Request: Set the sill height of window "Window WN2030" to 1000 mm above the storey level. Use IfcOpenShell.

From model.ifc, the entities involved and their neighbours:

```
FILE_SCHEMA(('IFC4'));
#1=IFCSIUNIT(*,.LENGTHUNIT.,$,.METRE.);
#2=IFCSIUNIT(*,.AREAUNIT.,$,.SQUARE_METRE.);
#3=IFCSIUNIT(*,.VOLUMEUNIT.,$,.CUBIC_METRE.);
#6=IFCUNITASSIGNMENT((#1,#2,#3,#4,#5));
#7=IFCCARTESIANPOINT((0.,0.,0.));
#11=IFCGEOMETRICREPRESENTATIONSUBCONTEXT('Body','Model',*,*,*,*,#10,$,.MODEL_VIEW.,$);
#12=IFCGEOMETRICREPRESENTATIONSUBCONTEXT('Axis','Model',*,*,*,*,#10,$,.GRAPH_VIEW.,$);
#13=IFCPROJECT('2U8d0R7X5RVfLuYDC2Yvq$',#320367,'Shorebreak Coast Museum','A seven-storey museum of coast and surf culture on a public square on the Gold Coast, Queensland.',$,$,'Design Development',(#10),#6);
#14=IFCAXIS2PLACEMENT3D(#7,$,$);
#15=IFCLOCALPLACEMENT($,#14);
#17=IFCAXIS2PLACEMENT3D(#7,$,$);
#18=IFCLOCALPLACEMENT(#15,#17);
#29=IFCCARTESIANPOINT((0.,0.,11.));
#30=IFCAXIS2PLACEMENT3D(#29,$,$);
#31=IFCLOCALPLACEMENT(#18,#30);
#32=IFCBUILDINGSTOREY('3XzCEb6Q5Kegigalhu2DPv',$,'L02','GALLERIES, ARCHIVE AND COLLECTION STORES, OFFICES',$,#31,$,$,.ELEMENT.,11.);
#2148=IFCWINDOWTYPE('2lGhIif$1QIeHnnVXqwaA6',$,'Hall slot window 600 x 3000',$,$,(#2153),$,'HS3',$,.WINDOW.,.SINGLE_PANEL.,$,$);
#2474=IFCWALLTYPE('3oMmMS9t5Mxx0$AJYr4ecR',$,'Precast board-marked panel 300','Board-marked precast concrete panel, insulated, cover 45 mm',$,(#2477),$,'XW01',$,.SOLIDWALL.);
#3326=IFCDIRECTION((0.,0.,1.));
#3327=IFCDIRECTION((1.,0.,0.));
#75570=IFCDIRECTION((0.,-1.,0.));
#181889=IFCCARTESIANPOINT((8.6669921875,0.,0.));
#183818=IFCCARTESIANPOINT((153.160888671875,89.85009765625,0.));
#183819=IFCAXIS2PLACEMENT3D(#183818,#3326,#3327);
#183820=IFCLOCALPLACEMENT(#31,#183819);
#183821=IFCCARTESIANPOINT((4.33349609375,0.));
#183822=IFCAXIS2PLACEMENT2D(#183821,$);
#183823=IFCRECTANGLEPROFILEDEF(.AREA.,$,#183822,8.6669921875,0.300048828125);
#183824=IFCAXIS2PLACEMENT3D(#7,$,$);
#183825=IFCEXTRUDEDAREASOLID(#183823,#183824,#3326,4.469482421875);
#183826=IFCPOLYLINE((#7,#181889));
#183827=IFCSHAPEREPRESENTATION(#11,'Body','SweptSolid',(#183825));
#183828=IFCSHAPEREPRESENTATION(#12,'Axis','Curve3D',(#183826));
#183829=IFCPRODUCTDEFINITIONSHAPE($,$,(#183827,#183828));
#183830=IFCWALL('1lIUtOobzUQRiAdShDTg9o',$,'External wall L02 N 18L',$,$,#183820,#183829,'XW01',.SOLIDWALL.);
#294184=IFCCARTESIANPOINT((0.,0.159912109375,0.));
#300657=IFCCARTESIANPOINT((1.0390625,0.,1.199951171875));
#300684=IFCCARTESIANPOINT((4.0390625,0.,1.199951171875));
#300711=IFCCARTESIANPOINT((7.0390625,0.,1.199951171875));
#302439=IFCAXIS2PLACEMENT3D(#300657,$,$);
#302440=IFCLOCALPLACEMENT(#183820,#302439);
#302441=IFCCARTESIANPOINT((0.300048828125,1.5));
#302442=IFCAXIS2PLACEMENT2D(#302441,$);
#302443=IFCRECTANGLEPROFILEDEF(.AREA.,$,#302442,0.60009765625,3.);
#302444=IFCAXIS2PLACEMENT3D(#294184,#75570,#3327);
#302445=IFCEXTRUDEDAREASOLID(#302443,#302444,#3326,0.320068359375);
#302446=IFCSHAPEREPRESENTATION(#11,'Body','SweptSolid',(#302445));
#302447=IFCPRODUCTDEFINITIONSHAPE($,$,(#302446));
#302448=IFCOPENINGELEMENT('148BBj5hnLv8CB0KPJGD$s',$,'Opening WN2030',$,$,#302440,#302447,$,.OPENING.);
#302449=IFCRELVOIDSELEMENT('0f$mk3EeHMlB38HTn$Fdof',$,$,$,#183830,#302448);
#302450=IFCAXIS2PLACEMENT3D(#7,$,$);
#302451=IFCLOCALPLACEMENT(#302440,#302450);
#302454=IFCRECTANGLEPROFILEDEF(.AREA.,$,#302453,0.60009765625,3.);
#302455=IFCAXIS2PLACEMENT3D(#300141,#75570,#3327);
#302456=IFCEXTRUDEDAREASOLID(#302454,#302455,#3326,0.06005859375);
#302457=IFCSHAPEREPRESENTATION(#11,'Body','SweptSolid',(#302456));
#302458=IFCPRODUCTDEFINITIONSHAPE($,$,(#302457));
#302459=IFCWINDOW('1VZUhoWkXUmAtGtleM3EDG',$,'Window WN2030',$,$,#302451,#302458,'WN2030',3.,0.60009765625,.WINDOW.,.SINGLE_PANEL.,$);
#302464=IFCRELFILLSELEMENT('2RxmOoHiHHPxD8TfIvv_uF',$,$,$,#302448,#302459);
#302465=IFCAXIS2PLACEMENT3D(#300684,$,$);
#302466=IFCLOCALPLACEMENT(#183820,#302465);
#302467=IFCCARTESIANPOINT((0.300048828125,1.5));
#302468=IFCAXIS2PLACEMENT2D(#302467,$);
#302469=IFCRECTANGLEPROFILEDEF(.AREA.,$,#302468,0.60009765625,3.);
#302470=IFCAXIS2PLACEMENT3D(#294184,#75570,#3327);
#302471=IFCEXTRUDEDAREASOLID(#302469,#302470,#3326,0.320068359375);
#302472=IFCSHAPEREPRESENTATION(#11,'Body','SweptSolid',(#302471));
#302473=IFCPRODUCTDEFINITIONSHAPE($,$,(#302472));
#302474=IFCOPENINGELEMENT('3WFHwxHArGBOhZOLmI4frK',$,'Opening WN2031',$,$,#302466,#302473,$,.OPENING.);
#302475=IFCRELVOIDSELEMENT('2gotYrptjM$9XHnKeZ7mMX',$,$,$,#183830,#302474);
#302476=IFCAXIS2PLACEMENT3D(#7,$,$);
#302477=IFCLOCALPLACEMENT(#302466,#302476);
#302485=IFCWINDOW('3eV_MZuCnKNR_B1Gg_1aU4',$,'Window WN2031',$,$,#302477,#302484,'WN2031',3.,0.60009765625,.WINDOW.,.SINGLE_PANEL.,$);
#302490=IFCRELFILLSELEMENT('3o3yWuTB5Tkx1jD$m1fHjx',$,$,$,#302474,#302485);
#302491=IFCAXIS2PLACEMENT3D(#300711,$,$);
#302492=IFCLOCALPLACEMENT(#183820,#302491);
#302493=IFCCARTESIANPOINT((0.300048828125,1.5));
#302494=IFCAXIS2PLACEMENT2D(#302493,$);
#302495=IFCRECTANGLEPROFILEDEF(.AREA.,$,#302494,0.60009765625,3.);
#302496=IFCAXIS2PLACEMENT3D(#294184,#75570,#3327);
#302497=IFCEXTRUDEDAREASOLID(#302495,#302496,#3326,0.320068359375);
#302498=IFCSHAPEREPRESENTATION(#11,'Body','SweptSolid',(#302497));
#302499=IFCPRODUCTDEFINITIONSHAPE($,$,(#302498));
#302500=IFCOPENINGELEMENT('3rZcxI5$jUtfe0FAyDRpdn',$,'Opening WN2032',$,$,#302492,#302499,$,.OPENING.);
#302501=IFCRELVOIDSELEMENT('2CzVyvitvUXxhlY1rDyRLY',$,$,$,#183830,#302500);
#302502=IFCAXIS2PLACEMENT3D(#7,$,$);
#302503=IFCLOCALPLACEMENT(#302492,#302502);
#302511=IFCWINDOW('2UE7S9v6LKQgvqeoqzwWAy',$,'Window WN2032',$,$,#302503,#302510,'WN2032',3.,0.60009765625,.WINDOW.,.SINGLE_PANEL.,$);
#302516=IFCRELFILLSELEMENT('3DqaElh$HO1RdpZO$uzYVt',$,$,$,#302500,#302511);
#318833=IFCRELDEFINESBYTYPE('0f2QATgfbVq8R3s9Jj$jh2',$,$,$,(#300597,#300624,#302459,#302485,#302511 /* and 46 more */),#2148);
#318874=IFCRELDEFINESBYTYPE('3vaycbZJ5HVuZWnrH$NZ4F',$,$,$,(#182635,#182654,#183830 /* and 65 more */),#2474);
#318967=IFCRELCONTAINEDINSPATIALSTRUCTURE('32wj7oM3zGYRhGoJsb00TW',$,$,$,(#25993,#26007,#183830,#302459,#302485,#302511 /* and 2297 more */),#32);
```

```python
import numpy as np
import ifcopenshell
import ifcopenshell.api.geometry
import ifcopenshell.geom
import ifcopenshell.util.element
import ifcopenshell.util.placement
import ifcopenshell.util.shape
import ifcopenshell.util.unit

model = ifcopenshell.open("model.ifc")
unit_scale = ifcopenshell.util.unit.calculate_unit_scale(model)

window = model.by_guid("1VZUhoWkXUmAtGtleM3EDG")
opening = window.FillsVoids[0].RelatingOpeningElement
storey = ifcopenshell.util.element.get_container(window, ifc_class="IfcBuildingStorey")
level = ifcopenshell.util.placement.get_local_placement(storey.ObjectPlacement)[2, 3]

# The opening's origin need not be at the sill, so measure its lowest point.
shape = ifcopenshell.geom.create_shape(ifcopenshell.geom.settings(), opening)
bottom = ifcopenshell.util.shape.get_shape_bottom_elevation(shape, shape.geometry) / unit_scale
dz = level + 1.0 - bottom

shift = np.array([0.0, 0.0, dz])
# The window is placed relative to its opening, so it follows when the opening moves.
matrix = ifcopenshell.util.placement.get_local_placement(opening.ObjectPlacement)
matrix[:3, 3] += shift
ifcopenshell.api.geometry.edit_object_placement(
    model, product=opening, matrix=matrix, is_si=False, should_transform_children=True
)

print(f"moved by {dz * unit_scale:+.3f} m")

model.write("model-out.ifc")
```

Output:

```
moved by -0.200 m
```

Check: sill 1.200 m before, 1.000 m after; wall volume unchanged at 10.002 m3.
